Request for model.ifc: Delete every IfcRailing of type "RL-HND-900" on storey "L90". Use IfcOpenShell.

First a look at what the model holds.

```python
import ifcopenshell
import ifcopenshell.util.element

model = ifcopenshell.open("model.ifc")
print(model.schema)
storey = next(s for s in model.by_type("IfcBuildingStorey") if s.Name == "L90")
railings = [e for e in ifcopenshell.util.element.get_decomposition(storey) if e.is_a("IfcRailing")]
seen = {}
for e in railings:
    element_type = ifcopenshell.util.element.get_type(e)
    name = element_type.Name if element_type not in (None, e) else None
    seen[name] = seen.get(name, 0) + 1
for name, count in sorted(seen.items(), key=str):
    print(count, "x", name)
```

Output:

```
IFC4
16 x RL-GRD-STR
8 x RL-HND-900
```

```python
import ifcopenshell
import ifcopenshell.api.root
import ifcopenshell.util.element

model = ifcopenshell.open("model.ifc")

storey = next(s for s in model.by_type("IfcBuildingStorey") if s.Name == "L90")
railings = [e for e in ifcopenshell.util.element.get_decomposition(storey) if e.is_a("IfcRailing")]
targets = [e for e in railings if (t := ifcopenshell.util.element.get_type(e)) not in (None, e) and t.Name == "RL-HND-900"]

for e in targets:
    ifcopenshell.api.root.remove_product(model, product=e)
print(len(targets), "removed")

model.write("model-out.ifc")
```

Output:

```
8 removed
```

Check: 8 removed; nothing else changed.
